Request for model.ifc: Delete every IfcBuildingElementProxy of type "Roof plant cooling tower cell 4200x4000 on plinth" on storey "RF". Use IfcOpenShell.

First a look at what the model holds.

```python
import ifcopenshell
import ifcopenshell.util.element

model = ifcopenshell.open("model.ifc")
print(model.schema)
storey = next(s for s in model.by_type("IfcBuildingStorey") if s.Name == "RF")
proxies = [e for e in ifcopenshell.util.element.get_decomposition(storey) if e.is_a("IfcBuildingElementProxy")]
seen = {}
for e in proxies:
    element_type = ifcopenshell.util.element.get_type(e)
    name = element_type.Name if element_type not in (None, e) else None
    seen[name] = seen.get(name, 0) + 1
for name, count in sorted(seen.items(), key=str):
    print(count, "x", name)
```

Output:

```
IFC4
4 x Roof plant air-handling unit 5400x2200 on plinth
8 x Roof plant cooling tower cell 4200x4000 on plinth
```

```python
import ifcopenshell
import ifcopenshell.api.root
import ifcopenshell.util.element

model = ifcopenshell.open("model.ifc")

storey = next(s for s in model.by_type("IfcBuildingStorey") if s.Name == "RF")
proxies = [e for e in ifcopenshell.util.element.get_decomposition(storey) if e.is_a("IfcBuildingElementProxy")]
targets = [e for e in proxies if (t := ifcopenshell.util.element.get_type(e)) not in (None, e) and t.Name == "Roof plant cooling tower cell 4200x4000 on plinth"]

for e in targets:
    ifcopenshell.api.root.remove_product(model, product=e)
print(len(targets), "removed")

model.write("model_updated.ifc")
```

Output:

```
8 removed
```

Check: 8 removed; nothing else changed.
